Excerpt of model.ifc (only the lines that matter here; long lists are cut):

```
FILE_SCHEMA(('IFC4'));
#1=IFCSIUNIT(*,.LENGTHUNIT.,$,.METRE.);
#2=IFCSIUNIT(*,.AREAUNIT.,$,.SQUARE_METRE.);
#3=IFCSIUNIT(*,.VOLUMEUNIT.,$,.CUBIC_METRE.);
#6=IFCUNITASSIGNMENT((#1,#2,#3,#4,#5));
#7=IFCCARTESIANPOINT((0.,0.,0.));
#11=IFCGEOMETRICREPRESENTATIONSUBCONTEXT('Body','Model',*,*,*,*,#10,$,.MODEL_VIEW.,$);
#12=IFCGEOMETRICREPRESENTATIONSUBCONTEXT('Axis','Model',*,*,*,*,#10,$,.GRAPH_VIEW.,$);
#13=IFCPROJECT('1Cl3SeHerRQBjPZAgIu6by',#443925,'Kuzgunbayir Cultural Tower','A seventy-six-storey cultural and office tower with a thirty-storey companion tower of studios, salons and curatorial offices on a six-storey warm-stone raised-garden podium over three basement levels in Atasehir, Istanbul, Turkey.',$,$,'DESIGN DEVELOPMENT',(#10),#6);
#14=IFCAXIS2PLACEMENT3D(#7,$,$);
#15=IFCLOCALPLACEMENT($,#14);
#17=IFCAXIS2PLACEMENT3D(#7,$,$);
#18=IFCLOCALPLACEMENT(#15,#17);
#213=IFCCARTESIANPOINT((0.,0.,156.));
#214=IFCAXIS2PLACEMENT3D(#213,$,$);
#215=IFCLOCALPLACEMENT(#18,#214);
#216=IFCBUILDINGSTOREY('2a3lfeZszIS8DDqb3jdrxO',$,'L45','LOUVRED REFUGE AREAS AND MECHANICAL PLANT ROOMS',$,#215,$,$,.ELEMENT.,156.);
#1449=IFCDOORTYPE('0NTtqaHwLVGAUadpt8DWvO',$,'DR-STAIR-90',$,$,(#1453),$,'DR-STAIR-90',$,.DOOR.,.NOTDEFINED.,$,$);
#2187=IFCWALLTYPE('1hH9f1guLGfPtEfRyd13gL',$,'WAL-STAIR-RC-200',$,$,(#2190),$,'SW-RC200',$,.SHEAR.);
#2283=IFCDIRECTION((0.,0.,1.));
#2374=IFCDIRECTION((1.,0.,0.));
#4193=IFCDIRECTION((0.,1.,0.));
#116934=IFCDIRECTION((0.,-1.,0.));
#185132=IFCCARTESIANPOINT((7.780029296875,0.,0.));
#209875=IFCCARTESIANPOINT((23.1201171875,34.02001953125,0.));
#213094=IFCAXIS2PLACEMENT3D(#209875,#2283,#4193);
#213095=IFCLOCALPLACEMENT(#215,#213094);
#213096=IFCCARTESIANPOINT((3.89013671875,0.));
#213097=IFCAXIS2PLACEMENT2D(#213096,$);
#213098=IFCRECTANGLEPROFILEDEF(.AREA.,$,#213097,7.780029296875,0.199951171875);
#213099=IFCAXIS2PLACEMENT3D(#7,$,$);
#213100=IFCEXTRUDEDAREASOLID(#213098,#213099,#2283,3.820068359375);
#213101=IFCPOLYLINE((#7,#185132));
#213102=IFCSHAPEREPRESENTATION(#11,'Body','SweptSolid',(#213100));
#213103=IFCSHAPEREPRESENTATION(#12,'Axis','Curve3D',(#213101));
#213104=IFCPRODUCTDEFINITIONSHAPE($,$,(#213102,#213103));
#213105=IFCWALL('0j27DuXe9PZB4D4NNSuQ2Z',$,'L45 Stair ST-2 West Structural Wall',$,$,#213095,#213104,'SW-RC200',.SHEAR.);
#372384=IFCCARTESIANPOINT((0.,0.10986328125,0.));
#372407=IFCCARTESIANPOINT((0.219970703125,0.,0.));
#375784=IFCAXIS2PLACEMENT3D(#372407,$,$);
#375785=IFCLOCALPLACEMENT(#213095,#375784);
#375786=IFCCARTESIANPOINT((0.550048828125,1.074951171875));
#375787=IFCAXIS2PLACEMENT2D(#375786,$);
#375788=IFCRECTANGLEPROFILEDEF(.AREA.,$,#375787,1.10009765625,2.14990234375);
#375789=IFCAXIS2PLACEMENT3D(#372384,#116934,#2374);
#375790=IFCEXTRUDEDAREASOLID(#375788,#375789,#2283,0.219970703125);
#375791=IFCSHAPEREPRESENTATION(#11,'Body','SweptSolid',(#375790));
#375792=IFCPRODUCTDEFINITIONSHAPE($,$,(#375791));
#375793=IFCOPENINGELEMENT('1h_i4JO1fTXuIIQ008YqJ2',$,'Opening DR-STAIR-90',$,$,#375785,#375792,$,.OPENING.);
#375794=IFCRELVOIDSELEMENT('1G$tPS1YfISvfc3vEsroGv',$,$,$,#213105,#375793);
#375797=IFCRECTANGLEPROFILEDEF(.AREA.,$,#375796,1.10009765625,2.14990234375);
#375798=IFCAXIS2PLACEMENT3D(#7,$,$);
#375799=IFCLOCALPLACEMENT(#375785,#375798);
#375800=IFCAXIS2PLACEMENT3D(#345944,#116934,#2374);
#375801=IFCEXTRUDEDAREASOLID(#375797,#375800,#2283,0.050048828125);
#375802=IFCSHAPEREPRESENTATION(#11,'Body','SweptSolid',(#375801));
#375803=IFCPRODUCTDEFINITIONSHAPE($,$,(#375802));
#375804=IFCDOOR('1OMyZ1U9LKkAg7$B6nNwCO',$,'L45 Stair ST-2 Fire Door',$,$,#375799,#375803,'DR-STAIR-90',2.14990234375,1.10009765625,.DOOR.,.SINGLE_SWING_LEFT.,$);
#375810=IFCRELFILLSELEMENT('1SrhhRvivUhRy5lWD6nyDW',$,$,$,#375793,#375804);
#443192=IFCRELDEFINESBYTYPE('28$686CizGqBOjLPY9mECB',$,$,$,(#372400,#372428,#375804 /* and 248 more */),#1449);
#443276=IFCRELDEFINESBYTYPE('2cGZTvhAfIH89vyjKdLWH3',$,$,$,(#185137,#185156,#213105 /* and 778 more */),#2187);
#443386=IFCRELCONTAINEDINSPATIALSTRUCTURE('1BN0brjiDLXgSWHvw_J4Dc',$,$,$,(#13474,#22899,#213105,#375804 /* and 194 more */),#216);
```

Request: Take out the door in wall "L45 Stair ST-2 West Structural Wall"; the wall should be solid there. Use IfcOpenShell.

```python
import ifcopenshell
import ifcopenshell.api.feature
import ifcopenshell.api.root
import ifcopenshell.geom
import ifcopenshell.util.shape

model = ifcopenshell.open("model.ifc")
settings = ifcopenshell.geom.settings()


def volume(element):
    """Net volume in cubic metres, openings subtracted."""
    shape = ifcopenshell.geom.create_shape(settings, element)
    return ifcopenshell.util.shape.get_volume(shape.geometry)


door = model.by_guid("1OMyZ1U9LKkAg7$B6nNwCO")
opening = door.FillsVoids[0].RelatingOpeningElement
wall = opening.VoidsElements[0].RelatingBuildingElement
before = volume(wall)

ifcopenshell.api.root.remove_product(model, product=door)
ifcopenshell.api.feature.remove_feature(model, feature=opening)

after = volume(wall)

print(f"wall volume {before:.3f} -> {after:.3f} m3")

model.write("model_v2.ifc")
```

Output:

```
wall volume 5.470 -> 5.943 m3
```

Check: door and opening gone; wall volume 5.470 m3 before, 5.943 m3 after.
